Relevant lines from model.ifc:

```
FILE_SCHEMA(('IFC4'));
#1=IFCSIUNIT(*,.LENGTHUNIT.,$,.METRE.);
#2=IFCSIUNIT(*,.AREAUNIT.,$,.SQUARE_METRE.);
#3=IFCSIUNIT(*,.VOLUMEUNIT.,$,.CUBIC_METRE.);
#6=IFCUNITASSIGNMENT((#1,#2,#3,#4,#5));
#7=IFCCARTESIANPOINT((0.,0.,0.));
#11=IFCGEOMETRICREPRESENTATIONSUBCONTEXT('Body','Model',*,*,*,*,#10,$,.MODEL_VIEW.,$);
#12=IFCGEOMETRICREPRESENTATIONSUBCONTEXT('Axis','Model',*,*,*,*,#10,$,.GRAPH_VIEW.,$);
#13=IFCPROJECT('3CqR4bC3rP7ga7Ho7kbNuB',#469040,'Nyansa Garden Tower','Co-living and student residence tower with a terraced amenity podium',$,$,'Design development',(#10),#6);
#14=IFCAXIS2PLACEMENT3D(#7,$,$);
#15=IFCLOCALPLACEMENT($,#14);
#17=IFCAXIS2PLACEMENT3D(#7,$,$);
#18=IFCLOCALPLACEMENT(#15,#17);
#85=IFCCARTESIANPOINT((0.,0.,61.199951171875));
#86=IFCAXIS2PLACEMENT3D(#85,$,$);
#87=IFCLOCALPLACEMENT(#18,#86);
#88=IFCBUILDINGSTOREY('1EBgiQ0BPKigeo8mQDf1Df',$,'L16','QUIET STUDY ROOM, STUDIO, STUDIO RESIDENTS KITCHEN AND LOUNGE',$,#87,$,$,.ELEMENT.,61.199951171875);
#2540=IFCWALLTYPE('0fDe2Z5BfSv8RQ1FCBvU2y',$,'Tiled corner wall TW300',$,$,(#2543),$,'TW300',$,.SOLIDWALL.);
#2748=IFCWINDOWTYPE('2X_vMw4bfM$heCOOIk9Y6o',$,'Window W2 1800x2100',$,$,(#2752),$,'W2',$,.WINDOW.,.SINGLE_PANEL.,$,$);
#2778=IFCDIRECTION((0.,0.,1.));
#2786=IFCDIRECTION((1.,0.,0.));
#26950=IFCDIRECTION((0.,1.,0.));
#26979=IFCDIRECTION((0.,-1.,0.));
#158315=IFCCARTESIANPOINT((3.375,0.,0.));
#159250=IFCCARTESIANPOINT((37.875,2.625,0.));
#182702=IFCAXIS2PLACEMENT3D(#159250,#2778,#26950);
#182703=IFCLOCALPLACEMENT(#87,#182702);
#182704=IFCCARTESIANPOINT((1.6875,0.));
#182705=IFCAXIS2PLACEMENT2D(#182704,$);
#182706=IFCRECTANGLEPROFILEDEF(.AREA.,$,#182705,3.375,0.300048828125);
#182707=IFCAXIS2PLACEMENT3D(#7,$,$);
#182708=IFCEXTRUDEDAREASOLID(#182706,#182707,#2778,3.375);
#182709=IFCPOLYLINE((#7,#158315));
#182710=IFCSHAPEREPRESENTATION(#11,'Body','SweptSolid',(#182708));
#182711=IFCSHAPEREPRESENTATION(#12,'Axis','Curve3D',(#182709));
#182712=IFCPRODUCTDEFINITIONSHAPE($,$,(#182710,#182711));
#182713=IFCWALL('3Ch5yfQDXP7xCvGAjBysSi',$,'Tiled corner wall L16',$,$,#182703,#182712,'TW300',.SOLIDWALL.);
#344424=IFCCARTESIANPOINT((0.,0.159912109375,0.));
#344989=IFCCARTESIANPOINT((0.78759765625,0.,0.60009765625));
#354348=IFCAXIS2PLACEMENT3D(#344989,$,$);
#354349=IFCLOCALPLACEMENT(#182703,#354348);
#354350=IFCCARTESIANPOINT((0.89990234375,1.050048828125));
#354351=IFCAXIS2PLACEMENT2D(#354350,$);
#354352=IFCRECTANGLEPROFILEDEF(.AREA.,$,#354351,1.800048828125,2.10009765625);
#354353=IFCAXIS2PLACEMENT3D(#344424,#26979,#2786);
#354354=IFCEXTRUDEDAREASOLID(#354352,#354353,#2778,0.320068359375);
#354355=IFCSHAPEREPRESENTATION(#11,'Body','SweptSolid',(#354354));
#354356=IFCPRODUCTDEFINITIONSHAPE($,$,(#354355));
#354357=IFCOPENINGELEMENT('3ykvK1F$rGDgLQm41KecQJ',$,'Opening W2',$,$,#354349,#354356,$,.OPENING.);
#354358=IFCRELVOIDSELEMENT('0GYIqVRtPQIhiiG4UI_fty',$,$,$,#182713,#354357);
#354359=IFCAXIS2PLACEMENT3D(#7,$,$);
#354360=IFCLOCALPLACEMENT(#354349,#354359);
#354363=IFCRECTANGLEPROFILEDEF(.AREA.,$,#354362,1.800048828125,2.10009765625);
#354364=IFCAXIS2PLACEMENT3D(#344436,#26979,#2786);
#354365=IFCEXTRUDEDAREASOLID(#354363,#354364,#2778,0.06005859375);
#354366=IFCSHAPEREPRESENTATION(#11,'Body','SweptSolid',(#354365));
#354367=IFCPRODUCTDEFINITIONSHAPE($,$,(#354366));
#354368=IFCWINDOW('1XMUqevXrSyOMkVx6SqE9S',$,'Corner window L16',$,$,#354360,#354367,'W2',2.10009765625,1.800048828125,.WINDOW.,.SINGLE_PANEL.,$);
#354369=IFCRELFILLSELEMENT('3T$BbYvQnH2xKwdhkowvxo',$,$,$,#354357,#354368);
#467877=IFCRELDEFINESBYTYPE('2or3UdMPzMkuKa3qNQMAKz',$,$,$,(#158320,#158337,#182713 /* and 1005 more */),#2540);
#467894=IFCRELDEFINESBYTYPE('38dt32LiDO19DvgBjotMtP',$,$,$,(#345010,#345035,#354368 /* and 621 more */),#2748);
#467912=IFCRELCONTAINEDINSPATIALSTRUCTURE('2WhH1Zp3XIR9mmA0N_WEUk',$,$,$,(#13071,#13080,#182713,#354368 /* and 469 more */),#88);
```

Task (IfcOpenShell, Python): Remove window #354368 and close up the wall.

```python
import ifcopenshell
import ifcopenshell.api.feature
import ifcopenshell.api.root
import ifcopenshell.geom
import ifcopenshell.util.shape

model = ifcopenshell.open("model.ifc")
settings = ifcopenshell.geom.settings()


def volume(element):
    """Net volume in cubic metres, openings subtracted."""
    shape = ifcopenshell.geom.create_shape(settings, element)
    return ifcopenshell.util.shape.get_volume(shape.geometry)


window = model.by_id(354368)
opening = window.FillsVoids[0].RelatingOpeningElement
wall = opening.VoidsElements[0].RelatingBuildingElement
before = volume(wall)

ifcopenshell.api.root.remove_product(model, product=window)
ifcopenshell.api.feature.remove_feature(model, feature=opening)

after = volume(wall)

print(f"wall volume {before:.3f} -> {after:.3f} m3")

model.write("model-out.ifc")
```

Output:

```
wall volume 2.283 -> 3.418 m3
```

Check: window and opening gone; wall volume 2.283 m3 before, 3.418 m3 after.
